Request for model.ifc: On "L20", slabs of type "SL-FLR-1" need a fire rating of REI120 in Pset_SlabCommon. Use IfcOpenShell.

First a look at what the model holds.

```python
import ifcopenshell
import ifcopenshell.util.element

model = ifcopenshell.open("model.ifc")
print(model.schema)
storey = next(s for s in model.by_type("IfcBuildingStorey") if s.Name == "L20")
slabs = [e for e in ifcopenshell.util.element.get_decomposition(storey) if e.is_a("IfcSlab")]
seen = {}
for e in slabs:
    element_type = ifcopenshell.util.element.get_type(e)
    key = (element_type.Name if element_type != e and element_type else None, ifcopenshell.util.element.get_pset(e, "Pset_SlabCommon", "FireRating"))
    seen[key] = seen.get(key, 0) + 1
for (name, value), count in sorted(seen.items(), key=str):
    print(count, "x", name, "|", value)
```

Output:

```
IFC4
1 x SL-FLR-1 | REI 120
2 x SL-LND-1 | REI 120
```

```python
import ifcopenshell
import ifcopenshell.api.pset
import ifcopenshell.util.element

model = ifcopenshell.open("model.ifc")

storey = next(s for s in model.by_type("IfcBuildingStorey") if s.Name == "L20")
slabs = [e for e in ifcopenshell.util.element.get_decomposition(storey) if e.is_a("IfcSlab")]

count = 0
for e in slabs:
    element_type = ifcopenshell.util.element.get_type(e)
    if element_type in (None, e) or element_type.Name != "SL-FLR-1":
        continue
    # add_pset returns the element's existing set when there is one.
    pset = ifcopenshell.api.pset.add_pset(model, product=e, name="Pset_SlabCommon")
    ifcopenshell.api.pset.edit_pset(model, pset=pset, properties={"FireRating": "REI120"})
    count += 1

print(count, "slabs updated")

model.write("model_edited.ifc")
```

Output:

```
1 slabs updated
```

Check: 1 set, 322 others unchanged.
